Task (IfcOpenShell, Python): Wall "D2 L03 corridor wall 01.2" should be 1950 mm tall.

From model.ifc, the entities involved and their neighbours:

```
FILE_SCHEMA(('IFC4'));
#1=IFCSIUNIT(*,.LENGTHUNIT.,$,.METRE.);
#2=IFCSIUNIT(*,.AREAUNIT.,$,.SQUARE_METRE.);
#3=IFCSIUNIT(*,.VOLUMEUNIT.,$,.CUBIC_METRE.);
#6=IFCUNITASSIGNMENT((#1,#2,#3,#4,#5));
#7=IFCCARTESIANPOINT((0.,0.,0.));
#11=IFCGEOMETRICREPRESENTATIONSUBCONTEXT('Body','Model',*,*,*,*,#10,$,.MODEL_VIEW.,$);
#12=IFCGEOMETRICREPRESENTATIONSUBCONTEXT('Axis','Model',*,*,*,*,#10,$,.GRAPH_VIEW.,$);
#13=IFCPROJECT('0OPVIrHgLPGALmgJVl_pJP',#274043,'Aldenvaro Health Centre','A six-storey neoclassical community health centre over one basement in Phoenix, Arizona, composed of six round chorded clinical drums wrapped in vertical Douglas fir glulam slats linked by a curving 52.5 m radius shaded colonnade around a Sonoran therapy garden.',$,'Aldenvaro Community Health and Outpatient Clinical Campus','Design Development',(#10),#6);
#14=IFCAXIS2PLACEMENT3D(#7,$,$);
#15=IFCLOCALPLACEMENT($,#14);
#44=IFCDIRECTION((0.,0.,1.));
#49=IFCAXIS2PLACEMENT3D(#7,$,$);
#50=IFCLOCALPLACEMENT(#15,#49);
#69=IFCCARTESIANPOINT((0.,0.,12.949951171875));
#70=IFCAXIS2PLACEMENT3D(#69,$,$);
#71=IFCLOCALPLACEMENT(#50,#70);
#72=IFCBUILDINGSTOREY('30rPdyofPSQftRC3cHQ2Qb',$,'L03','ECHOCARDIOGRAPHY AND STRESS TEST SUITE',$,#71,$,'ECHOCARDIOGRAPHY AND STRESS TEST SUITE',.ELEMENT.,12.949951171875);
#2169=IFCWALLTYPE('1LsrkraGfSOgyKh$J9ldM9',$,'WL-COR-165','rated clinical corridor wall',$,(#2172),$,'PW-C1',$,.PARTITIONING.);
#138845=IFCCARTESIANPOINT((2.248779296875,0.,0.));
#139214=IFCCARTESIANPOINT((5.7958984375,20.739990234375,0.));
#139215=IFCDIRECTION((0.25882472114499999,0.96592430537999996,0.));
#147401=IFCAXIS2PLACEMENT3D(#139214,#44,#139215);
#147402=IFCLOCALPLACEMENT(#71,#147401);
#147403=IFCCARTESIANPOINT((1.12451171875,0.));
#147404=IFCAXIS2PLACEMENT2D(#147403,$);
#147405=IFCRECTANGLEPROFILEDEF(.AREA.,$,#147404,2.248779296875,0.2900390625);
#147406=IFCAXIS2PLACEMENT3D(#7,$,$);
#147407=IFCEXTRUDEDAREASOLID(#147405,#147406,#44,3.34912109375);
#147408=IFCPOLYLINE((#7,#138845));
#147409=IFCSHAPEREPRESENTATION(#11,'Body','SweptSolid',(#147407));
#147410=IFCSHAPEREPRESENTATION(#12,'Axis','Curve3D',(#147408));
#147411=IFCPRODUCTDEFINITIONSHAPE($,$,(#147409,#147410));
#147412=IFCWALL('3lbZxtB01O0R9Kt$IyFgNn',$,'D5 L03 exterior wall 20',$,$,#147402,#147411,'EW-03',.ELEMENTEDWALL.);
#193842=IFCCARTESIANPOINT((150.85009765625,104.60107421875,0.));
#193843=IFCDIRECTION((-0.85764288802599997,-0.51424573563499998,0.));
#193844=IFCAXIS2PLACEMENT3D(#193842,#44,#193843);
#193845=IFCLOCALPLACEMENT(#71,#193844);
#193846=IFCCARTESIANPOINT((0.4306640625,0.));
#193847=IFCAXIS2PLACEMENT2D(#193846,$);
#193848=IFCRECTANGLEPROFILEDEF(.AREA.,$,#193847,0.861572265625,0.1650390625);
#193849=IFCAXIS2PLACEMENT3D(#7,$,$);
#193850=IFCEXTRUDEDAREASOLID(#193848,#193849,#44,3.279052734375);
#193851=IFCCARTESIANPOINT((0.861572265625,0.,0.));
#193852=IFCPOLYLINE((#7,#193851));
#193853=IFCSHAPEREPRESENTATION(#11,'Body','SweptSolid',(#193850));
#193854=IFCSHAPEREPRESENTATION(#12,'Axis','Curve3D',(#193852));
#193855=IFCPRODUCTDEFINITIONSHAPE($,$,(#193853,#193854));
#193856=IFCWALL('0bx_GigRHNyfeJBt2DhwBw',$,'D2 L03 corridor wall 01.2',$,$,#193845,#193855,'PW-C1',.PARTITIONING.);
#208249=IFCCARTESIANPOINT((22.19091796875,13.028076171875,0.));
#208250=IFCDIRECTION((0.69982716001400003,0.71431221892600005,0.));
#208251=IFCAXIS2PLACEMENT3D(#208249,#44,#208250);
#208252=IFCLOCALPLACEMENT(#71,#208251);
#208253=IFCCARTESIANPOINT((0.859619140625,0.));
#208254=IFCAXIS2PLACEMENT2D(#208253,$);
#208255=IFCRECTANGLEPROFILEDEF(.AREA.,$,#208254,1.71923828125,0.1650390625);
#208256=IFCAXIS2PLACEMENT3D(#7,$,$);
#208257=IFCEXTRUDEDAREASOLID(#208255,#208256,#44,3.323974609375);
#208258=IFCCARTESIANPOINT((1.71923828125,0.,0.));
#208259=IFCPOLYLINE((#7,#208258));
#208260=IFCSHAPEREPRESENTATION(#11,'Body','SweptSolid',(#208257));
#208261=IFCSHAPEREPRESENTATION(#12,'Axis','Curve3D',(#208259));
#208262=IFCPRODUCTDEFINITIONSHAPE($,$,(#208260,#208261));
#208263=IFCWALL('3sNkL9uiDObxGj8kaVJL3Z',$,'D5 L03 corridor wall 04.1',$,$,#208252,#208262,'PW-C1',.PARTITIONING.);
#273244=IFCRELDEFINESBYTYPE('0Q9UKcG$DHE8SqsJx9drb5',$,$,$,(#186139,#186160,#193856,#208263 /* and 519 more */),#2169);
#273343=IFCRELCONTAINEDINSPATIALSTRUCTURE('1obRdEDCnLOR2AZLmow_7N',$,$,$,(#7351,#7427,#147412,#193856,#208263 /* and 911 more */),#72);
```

```python
import ifcopenshell
import ifcopenshell.geom
import ifcopenshell.util.representation
import ifcopenshell.util.shape
import ifcopenshell.util.unit

model = ifcopenshell.open("model.ifc")
unit_scale = ifcopenshell.util.unit.calculate_unit_scale(model)
settings = ifcopenshell.geom.settings()


def volume(element):
    """Net volume in cubic metres, openings subtracted."""
    shape = ifcopenshell.geom.create_shape(settings, element)
    return ifcopenshell.util.shape.get_volume(shape.geometry)


wall = model.by_guid("0bx_GigRHNyfeJBt2DhwBw")
before = volume(wall)

body = ifcopenshell.util.representation.get_representation(wall, "Model", "Body")
solid = body.Items[0]
old_height = solid.Depth
solid.Depth = 1.95 / unit_scale
after = volume(wall)

print(f"height {old_height:g} -> {solid.Depth:g}, volume {before:.3f} -> {after:.3f} m3")

model.write("model_v2.ifc")
```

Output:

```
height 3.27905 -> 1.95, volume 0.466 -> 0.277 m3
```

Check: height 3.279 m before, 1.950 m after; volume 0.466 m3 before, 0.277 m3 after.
